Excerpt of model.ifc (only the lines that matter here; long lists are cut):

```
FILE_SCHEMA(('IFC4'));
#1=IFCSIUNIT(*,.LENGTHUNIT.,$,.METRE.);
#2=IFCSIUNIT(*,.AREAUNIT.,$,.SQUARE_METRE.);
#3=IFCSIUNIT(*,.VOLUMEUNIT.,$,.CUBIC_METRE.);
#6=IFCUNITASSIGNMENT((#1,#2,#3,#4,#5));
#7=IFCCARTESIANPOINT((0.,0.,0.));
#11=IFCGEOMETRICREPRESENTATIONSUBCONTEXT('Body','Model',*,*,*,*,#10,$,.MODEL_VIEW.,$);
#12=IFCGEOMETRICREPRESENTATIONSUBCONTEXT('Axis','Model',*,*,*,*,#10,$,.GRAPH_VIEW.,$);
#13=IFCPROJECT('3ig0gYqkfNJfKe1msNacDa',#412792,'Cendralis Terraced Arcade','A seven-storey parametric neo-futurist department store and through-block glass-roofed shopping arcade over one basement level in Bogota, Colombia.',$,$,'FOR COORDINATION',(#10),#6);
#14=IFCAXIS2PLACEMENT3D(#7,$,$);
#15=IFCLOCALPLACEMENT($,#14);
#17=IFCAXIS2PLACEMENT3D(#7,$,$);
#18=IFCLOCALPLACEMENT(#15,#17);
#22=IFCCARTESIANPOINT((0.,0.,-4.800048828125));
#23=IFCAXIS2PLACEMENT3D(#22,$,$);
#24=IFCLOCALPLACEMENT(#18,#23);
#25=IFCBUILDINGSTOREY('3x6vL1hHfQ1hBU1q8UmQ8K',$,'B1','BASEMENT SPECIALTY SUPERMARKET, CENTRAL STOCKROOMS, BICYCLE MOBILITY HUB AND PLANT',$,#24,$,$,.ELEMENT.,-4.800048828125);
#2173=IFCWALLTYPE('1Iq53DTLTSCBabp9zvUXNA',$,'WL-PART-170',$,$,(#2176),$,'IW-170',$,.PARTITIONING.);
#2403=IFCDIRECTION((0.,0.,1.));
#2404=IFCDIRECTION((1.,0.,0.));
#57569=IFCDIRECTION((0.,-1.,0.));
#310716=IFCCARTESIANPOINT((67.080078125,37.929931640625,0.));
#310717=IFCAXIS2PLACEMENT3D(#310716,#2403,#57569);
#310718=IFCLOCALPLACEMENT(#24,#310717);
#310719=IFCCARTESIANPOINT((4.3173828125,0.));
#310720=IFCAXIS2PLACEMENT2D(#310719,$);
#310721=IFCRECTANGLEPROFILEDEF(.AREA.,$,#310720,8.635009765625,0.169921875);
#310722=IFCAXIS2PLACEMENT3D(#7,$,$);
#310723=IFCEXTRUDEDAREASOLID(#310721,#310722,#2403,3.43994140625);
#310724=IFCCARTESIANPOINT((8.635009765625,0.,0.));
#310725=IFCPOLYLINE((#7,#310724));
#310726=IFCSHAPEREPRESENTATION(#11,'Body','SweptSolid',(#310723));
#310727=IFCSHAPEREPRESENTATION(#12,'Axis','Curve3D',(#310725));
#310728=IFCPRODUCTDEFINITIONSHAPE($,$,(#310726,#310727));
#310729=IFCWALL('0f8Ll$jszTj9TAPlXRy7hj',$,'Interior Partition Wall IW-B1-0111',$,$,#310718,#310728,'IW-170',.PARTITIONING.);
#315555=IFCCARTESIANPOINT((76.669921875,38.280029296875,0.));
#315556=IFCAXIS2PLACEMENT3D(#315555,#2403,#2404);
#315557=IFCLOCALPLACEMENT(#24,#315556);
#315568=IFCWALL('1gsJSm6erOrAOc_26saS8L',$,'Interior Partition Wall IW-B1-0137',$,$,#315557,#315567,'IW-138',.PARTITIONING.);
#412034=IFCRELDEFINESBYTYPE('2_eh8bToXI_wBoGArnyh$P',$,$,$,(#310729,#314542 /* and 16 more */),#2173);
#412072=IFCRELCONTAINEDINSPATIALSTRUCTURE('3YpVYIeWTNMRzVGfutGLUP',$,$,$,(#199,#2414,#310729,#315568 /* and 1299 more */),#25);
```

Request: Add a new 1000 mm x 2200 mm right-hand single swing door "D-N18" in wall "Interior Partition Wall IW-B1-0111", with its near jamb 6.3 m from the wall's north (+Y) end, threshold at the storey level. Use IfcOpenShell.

```python
import numpy as np
import ifcopenshell
import ifcopenshell.api.feature
import ifcopenshell.api.geometry
import ifcopenshell.api.root
import ifcopenshell.api.spatial
import ifcopenshell.geom
import ifcopenshell.util.element
import ifcopenshell.util.placement
import ifcopenshell.util.representation
import ifcopenshell.util.shape
import ifcopenshell.util.unit

model = ifcopenshell.open("model.ifc")
unit_scale = ifcopenshell.util.unit.calculate_unit_scale(model)
settings = ifcopenshell.geom.settings()


def volume(element):
    """Net volume in cubic metres, openings subtracted."""
    shape = ifcopenshell.geom.create_shape(settings, element)
    return ifcopenshell.util.shape.get_volume(shape.geometry)


wall = model.by_id(310729)
storey = ifcopenshell.util.element.get_container(wall, ifc_class="IfcBuildingStorey")
context = ifcopenshell.util.representation.get_context(model, "Model", "Body", "MODEL_VIEW")
before = volume(wall)

width, height, from_end, sill = 1, 2.2, 6.3, 0.0  # metres

# The wall runs along its own X axis, and the end named is its -X end.
wall_shape = ifcopenshell.geom.create_shape(settings, wall)
x, y, z = ifcopenshell.util.shape.get_vertices(wall_shape.geometry).T
start = x.min() + from_end
face, thickness = float(y.min()), float(y.max() - y.min())
wall_matrix = ifcopenshell.util.placement.get_local_placement(wall.ObjectPlacement)
level = ifcopenshell.util.placement.get_local_placement(storey.ObjectPlacement)[2, 3]


def in_wall(x, y):
    """Placement at x, y metres in the wall's axes, at sill height."""
    matrix = wall_matrix.copy()
    matrix[:, 3] = wall_matrix @ np.array([x / unit_scale, y / unit_scale, 0.0, 1.0])
    matrix[2, 3] = level + sill / unit_scale
    return matrix


# Opening: a box that overshoots both wall faces by 50 mm.
opening = ifcopenshell.api.root.create_entity(model, ifc_class="IfcOpeningElement", predefined_type="OPENING")
box = ifcopenshell.api.geometry.add_wall_representation(
    model, context=context, length=width, height=height, thickness=thickness + 0.1
)
ifcopenshell.api.geometry.assign_representation(model, product=opening, representation=box)
ifcopenshell.api.geometry.edit_object_placement(model, product=opening, matrix=in_wall(start, face - 0.05), is_si=False)
ifcopenshell.api.feature.add_feature(model, feature=opening, element=wall)

door = ifcopenshell.api.root.create_entity(model, ifc_class="IfcDoor", name="D-N18", predefined_type="DOOR")
door.OverallWidth, door.OverallHeight = width / unit_scale, height / unit_scale
door.OperationType = "SINGLE_SWING_RIGHT"
body = ifcopenshell.api.geometry.add_door_representation(
    model,
    context=context,
    overall_width=door.OverallWidth,
    overall_height=door.OverallHeight,
    operation_type="SINGLE_SWING_RIGHT",
    lining_properties={"LiningDepth": thickness / unit_scale, "ThresholdDepth": thickness / unit_scale},
)
ifcopenshell.api.geometry.assign_representation(model, product=door, representation=body)
ifcopenshell.api.spatial.assign_container(model, products=[door], relating_structure=storey)
ifcopenshell.api.feature.add_filling(model, opening=opening, element=door)

# The lining spans the wall, so the door starts at the wall face.
ifcopenshell.api.geometry.edit_object_placement(model, product=door, matrix=in_wall(start, face), is_si=False)

after = volume(wall)

print(f"wall volume {before:.3f} -> {after:.3f} m3")

model.write("model-out.ifc")
```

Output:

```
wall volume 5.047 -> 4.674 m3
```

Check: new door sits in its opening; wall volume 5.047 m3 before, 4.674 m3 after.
